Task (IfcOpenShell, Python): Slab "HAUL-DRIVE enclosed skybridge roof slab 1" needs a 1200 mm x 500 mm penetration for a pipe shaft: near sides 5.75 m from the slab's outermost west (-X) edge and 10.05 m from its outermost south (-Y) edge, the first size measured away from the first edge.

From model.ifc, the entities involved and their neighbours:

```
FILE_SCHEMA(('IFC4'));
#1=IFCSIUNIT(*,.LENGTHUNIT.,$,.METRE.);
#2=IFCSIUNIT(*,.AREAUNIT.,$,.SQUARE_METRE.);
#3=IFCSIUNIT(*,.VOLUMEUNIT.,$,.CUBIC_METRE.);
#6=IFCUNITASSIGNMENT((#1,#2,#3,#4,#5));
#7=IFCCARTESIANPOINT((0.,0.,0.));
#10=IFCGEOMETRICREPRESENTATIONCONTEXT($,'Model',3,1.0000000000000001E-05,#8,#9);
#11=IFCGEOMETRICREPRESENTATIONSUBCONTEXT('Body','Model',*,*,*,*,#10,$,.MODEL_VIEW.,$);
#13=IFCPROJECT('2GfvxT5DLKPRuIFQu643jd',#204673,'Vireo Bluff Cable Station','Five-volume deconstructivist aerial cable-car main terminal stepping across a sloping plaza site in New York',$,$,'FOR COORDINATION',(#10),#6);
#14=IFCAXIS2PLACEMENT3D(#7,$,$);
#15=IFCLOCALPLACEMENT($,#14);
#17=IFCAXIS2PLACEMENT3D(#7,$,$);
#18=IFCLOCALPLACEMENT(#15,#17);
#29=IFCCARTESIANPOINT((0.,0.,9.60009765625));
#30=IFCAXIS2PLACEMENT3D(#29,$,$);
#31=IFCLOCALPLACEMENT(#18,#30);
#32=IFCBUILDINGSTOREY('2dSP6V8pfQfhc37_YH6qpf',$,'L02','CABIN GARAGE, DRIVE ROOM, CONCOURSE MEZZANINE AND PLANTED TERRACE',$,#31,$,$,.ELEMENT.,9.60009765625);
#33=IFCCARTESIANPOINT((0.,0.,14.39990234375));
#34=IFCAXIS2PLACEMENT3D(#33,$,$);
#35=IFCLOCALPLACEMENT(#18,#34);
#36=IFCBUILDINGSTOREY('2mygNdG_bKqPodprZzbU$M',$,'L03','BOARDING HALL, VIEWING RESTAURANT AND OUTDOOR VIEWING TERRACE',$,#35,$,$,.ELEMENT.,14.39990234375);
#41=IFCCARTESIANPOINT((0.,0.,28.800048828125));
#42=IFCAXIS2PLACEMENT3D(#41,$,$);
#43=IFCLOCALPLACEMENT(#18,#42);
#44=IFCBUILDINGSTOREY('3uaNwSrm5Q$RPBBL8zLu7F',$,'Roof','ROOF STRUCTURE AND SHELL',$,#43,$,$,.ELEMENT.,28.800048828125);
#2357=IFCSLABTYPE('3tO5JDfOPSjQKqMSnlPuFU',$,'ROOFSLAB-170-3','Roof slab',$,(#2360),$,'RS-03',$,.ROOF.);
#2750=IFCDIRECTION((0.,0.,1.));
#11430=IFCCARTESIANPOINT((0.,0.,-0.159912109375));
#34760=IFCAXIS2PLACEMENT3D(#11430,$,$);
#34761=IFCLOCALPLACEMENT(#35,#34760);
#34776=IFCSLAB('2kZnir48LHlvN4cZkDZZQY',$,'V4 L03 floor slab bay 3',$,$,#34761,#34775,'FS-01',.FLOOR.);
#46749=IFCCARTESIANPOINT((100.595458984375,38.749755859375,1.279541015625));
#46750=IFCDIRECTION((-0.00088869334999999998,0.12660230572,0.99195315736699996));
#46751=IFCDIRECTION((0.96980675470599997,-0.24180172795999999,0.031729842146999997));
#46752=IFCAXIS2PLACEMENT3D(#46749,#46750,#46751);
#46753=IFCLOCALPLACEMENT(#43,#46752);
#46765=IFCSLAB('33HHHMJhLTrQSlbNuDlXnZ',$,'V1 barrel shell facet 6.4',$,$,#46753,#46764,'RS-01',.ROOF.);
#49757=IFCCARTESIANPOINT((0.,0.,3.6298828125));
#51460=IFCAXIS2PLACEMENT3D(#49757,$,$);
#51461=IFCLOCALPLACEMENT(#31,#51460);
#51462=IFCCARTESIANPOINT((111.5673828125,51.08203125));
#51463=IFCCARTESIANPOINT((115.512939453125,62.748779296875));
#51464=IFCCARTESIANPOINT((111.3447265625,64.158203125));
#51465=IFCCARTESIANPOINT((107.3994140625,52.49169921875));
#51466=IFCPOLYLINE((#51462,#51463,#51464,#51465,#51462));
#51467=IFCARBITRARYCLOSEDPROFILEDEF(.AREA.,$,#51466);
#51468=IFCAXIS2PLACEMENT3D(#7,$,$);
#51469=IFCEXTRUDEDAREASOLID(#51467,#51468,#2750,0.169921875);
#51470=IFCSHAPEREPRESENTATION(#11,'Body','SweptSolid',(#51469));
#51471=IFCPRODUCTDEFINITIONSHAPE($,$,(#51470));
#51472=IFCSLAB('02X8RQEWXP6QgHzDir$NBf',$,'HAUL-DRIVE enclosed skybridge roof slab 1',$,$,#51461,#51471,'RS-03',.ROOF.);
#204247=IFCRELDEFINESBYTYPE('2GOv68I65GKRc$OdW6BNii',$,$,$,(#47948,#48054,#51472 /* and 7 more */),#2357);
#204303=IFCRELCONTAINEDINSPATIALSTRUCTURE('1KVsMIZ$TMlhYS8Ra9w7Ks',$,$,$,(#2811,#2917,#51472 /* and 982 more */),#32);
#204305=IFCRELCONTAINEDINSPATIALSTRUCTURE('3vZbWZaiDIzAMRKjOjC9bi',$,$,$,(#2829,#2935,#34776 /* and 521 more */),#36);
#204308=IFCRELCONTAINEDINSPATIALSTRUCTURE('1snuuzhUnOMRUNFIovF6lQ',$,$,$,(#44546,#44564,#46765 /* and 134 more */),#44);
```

```python
import numpy as np
import ifcopenshell
import ifcopenshell.api.feature
import ifcopenshell.api.geometry
import ifcopenshell.api.root
import ifcopenshell.geom
import ifcopenshell.util.placement
import ifcopenshell.util.representation
import ifcopenshell.util.shape
import ifcopenshell.util.unit

model = ifcopenshell.open("model.ifc")
unit_scale = ifcopenshell.util.unit.calculate_unit_scale(model)
settings = ifcopenshell.geom.settings()


def volume(element):
    """Net volume in cubic metres, openings subtracted."""
    shape = ifcopenshell.geom.create_shape(settings, element)
    return ifcopenshell.util.shape.get_volume(shape.geometry)


slab = model.by_id(51472)
before = volume(slab)

# Extent in the slab's own axes, in metres. The edges named are its -X and -Y sides.
slab_shape = ifcopenshell.geom.create_shape(settings, slab)
vertices = ifcopenshell.util.shape.get_vertices(slab_shape.geometry)
x_min, y_min, bottom = vertices.min(axis=0)
top = vertices[:, 2].max()

opening = ifcopenshell.api.root.create_entity(model, ifc_class="IfcOpeningElement", name="Pipe shaft opening", predefined_type="OPENING")
context = ifcopenshell.util.representation.get_context(model, "Model", "Body", "MODEL_VIEW")
width, depth = 1.2, 0.5
outline = [(0.0, 0.0), (width, 0.0), (width, depth), (0.0, depth), (0.0, 0.0)]
# Overshoot both faces by 50 mm so the cut is clean.
shape = ifcopenshell.api.geometry.add_slab_representation(
    model, context=context, depth=top - bottom + 0.1, polyline=outline
)
ifcopenshell.api.geometry.assign_representation(model, product=opening, representation=shape)

matrix = ifcopenshell.util.placement.get_local_placement(slab.ObjectPlacement)
matrix[:, 3] = matrix @ np.append(np.array([x_min + 5.75, y_min + 10.05, bottom - 0.05]) / unit_scale, 1.0)
ifcopenshell.api.geometry.edit_object_placement(model, product=opening, matrix=matrix, is_si=False)
ifcopenshell.api.feature.add_feature(model, feature=opening, element=slab)

after = volume(slab)

print(f"slab volume {before:.3f} -> {after:.3f} m3")

model.write("model-out.ifc")
```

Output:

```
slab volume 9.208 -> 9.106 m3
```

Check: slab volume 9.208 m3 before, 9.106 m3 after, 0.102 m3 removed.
